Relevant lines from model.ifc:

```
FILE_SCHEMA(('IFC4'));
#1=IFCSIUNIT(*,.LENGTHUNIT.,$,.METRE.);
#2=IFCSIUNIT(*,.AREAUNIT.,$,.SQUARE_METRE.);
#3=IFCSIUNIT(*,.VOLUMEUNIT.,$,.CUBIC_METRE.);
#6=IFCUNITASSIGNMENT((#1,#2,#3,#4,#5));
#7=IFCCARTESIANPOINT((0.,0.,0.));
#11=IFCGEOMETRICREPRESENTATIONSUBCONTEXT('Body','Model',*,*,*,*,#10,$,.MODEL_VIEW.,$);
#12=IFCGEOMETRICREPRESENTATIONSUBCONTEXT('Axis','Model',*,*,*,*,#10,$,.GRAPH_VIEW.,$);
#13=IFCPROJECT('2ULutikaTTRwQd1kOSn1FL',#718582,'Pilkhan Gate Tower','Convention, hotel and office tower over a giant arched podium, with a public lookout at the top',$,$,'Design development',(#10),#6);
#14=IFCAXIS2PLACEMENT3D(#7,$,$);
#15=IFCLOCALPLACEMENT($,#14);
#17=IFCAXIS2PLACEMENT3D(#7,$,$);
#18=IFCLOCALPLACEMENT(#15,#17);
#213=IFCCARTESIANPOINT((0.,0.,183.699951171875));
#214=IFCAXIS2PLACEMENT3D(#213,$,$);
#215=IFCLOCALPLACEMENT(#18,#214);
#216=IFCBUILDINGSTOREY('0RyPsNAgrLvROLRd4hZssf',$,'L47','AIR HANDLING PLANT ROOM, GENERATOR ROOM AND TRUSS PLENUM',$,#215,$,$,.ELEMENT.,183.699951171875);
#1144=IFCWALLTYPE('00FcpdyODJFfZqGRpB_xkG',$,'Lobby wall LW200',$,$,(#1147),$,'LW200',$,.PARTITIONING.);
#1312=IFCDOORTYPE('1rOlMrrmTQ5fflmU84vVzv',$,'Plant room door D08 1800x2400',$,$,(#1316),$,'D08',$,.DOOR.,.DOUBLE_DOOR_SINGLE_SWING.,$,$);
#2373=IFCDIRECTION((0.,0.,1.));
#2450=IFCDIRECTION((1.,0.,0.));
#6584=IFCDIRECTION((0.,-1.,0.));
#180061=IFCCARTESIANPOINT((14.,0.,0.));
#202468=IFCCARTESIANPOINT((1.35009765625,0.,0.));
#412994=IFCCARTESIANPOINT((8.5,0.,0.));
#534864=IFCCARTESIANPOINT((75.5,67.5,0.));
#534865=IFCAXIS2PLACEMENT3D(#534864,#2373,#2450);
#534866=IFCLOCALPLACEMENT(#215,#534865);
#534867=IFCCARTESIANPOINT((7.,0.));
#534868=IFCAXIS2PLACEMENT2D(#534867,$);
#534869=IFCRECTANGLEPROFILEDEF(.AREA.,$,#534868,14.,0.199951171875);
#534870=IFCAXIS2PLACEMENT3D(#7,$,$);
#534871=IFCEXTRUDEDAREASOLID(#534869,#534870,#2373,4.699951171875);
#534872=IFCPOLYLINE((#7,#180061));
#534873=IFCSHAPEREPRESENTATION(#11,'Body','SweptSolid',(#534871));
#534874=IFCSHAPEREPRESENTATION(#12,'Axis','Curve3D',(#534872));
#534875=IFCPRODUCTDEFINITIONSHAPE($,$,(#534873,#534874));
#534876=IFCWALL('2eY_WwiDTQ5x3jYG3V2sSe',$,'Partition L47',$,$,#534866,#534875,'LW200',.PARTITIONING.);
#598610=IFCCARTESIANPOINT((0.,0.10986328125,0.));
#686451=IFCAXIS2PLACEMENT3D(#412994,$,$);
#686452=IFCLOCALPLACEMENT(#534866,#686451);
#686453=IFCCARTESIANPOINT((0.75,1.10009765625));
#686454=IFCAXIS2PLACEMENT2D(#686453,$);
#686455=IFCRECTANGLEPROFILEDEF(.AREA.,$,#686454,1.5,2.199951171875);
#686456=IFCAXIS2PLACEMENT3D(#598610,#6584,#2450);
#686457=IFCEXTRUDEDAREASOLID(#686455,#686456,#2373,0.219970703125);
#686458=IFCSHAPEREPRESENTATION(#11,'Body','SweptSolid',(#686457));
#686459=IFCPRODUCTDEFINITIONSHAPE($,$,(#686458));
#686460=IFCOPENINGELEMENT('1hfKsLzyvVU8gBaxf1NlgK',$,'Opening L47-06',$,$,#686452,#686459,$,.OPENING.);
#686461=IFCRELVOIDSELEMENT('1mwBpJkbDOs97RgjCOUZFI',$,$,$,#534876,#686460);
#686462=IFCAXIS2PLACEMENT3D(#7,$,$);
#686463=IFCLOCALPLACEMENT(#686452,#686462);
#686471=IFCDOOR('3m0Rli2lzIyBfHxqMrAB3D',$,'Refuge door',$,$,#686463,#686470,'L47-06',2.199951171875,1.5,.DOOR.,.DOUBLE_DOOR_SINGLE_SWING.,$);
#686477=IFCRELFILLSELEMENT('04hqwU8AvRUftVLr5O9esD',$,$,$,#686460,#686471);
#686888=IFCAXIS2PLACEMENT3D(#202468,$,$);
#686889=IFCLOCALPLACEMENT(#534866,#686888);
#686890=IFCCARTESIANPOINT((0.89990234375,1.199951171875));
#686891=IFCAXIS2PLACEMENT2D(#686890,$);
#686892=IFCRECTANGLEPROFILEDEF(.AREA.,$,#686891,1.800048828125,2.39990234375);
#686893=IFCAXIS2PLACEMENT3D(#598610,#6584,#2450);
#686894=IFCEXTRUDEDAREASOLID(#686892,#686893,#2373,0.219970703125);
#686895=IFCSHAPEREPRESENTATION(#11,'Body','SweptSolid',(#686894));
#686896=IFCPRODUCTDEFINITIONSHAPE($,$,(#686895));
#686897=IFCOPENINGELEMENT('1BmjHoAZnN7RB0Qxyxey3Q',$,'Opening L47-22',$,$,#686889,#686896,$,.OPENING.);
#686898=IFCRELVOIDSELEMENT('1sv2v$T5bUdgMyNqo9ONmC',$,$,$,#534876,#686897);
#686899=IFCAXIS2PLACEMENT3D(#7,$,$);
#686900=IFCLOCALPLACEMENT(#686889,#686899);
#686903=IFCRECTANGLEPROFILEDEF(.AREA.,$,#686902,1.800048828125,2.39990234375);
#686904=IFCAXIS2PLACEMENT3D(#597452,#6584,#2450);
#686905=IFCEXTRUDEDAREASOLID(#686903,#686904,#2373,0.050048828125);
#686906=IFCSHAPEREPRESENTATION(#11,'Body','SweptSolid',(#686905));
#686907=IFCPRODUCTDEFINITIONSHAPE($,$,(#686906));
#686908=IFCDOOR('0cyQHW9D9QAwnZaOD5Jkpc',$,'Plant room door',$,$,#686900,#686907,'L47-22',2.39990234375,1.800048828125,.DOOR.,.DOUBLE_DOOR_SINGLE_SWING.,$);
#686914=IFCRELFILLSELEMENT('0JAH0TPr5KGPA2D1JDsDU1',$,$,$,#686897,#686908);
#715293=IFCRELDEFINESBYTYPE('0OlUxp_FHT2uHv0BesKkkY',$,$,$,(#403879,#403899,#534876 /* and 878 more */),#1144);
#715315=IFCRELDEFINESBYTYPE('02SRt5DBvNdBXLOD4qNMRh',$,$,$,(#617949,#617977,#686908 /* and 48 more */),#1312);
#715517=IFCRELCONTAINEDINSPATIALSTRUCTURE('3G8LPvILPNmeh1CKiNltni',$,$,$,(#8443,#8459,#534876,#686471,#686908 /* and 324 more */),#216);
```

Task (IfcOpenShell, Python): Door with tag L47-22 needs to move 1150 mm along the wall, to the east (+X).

```python
import ifcopenshell
import ifcopenshell.api.geometry
import ifcopenshell.util.placement

model = ifcopenshell.open("model.ifc")

door = model.by_guid("0cyQHW9D9QAwnZaOD5Jkpc")
opening = door.FillsVoids[0].RelatingOpeningElement
wall = opening.VoidsElements[0].RelatingBuildingElement

wall_matrix = ifcopenshell.util.placement.get_local_placement(wall.ObjectPlacement)
shift = wall_matrix[:3, 0] * 1.15
before = ifcopenshell.util.placement.get_local_placement(door.ObjectPlacement)[:3, 3].copy()

# The door is placed relative to its opening, so it follows when the opening moves.
matrix = ifcopenshell.util.placement.get_local_placement(opening.ObjectPlacement)
matrix[:3, 3] += shift
ifcopenshell.api.geometry.edit_object_placement(
    model, product=opening, matrix=matrix, is_si=False, should_transform_children=True
)

after = ifcopenshell.util.placement.get_local_placement(door.ObjectPlacement)[:3, 3]
print("door moved by", (after - before).round(3) + 0.0)

model.write("model_edited.ifc")
```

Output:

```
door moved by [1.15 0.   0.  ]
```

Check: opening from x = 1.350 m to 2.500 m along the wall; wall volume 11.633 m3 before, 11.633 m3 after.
